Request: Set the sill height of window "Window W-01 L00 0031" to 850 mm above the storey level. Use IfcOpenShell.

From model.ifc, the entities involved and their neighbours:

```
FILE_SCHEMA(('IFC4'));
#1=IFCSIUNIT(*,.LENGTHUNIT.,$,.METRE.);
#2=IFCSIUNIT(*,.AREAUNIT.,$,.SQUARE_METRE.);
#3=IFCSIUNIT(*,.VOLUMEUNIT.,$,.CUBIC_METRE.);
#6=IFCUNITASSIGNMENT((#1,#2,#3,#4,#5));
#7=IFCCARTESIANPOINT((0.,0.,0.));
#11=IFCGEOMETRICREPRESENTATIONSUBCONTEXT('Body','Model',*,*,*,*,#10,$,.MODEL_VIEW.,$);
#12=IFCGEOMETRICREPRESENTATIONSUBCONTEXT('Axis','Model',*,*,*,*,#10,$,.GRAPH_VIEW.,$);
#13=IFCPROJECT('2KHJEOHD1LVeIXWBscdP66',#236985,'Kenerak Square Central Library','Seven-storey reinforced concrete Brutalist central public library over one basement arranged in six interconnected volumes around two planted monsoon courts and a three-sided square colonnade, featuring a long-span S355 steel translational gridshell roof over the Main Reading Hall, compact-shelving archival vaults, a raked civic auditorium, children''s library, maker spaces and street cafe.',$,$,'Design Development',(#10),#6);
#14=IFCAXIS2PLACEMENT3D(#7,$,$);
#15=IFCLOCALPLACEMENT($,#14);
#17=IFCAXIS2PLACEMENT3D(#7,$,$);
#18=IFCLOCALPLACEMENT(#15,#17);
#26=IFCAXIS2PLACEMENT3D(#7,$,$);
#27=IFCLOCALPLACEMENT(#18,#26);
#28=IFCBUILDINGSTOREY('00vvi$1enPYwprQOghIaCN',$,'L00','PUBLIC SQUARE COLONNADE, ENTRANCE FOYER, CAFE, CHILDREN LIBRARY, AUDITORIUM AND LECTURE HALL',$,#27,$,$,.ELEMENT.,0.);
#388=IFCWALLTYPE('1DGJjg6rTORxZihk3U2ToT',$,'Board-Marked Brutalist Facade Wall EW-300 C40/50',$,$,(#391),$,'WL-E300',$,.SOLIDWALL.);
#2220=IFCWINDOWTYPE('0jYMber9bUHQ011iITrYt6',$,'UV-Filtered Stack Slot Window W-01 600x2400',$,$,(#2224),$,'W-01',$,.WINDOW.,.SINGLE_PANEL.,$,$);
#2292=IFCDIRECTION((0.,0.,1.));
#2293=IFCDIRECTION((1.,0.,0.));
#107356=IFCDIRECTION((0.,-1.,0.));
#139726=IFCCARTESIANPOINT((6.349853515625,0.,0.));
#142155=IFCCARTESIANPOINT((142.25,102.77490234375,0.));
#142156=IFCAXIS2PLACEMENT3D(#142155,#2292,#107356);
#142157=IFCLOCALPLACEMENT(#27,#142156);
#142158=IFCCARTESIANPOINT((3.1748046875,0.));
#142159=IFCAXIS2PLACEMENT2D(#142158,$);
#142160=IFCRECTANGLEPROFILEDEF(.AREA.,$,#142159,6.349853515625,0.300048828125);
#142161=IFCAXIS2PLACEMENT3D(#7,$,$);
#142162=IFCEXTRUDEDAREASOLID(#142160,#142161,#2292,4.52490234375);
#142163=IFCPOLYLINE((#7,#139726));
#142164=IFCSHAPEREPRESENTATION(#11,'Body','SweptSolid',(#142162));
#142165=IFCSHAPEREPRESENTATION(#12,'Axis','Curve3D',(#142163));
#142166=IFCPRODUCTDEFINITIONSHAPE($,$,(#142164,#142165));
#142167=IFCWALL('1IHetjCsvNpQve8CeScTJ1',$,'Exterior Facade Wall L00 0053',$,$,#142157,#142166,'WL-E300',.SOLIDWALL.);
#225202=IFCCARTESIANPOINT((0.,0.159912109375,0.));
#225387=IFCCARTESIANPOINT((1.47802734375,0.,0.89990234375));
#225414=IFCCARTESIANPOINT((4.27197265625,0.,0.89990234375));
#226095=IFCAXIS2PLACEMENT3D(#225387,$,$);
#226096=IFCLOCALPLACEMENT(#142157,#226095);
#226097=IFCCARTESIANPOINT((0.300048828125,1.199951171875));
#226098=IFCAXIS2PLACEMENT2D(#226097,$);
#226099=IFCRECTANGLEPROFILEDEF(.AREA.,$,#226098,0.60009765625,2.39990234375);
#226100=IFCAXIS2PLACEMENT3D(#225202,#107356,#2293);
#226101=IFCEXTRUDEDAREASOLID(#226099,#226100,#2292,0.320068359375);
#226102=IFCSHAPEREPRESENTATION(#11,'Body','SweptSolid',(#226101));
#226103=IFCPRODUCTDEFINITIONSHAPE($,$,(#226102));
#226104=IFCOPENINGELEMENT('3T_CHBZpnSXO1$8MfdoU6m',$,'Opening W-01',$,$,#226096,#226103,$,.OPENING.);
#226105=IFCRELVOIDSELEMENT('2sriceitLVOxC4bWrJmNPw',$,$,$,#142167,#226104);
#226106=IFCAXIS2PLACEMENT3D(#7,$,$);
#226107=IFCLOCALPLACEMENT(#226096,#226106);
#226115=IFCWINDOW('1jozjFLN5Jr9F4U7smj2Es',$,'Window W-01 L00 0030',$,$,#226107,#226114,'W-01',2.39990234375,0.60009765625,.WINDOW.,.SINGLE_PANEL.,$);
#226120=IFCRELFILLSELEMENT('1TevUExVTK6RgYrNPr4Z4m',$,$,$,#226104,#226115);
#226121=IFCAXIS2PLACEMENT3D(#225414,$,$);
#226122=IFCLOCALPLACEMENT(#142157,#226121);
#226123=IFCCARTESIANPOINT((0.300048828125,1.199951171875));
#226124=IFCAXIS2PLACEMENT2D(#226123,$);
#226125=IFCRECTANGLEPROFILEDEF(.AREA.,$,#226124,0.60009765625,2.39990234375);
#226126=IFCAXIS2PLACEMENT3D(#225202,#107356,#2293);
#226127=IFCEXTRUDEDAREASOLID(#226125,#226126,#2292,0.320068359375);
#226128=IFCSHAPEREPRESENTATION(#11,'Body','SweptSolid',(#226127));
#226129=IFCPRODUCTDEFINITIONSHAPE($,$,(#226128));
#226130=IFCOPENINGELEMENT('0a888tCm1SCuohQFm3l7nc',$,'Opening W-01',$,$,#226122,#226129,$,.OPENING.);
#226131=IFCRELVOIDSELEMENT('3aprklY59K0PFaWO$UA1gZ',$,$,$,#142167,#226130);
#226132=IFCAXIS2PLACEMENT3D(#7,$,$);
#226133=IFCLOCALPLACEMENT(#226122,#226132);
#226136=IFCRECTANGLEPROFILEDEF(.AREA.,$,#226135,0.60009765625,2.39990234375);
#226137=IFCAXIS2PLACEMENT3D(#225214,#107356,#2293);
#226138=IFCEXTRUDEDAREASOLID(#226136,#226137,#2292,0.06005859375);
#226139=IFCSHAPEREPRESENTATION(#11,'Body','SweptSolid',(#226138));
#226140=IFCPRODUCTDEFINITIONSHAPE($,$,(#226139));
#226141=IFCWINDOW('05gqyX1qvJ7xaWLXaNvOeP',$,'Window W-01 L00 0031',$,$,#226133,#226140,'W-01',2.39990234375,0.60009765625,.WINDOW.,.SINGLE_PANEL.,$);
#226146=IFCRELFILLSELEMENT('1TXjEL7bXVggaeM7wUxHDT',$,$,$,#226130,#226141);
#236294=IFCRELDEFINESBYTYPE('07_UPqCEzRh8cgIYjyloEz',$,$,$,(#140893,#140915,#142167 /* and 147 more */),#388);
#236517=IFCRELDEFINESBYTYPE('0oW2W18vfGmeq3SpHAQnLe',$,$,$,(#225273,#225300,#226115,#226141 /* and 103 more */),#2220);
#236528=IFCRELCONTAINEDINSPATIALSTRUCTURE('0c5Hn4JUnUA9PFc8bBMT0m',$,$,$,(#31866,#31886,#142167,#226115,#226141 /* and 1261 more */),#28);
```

```python
import numpy as np
import ifcopenshell
import ifcopenshell.api.geometry
import ifcopenshell.geom
import ifcopenshell.util.element
import ifcopenshell.util.placement
import ifcopenshell.util.shape
import ifcopenshell.util.unit

model = ifcopenshell.open("model.ifc")
unit_scale = ifcopenshell.util.unit.calculate_unit_scale(model)

window = model.by_id(226141)
opening = window.FillsVoids[0].RelatingOpeningElement
storey = ifcopenshell.util.element.get_container(window, ifc_class="IfcBuildingStorey")
level = ifcopenshell.util.placement.get_local_placement(storey.ObjectPlacement)[2, 3]

# The opening's origin need not be at the sill, so measure its lowest point.
shape = ifcopenshell.geom.create_shape(ifcopenshell.geom.settings(), opening)
bottom = ifcopenshell.util.shape.get_shape_bottom_elevation(shape, shape.geometry) / unit_scale
dz = level + 0.85 / unit_scale - bottom

shift = np.array([0.0, 0.0, dz])
# The window is placed relative to its opening, so it follows when the opening moves.
matrix = ifcopenshell.util.placement.get_local_placement(opening.ObjectPlacement)
matrix[:3, 3] += shift
ifcopenshell.api.geometry.edit_object_placement(
    model, product=opening, matrix=matrix, is_si=False, should_transform_children=True
)

print(f"moved by {dz * unit_scale:+.3f} m")

model.write("model_updated.ifc")
```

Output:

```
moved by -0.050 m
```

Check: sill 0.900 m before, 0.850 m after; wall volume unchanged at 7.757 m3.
